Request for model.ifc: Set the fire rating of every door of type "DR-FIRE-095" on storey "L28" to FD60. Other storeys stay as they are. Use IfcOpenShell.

First a look at what the model holds.

```python
import ifcopenshell
import ifcopenshell.util.element

model = ifcopenshell.open("model.ifc")
print(model.schema)
storey = next(s for s in model.by_type("IfcBuildingStorey") if s.Name == "L28")
doors = [e for e in ifcopenshell.util.element.get_decomposition(storey) if e.is_a("IfcDoor")]
seen = {}
for e in doors:
    element_type = ifcopenshell.util.element.get_type(e)
    key = (element_type.Name if element_type != e and element_type else None, ifcopenshell.util.element.get_pset(e, "Pset_DoorCommon", "FireRating"))
    seen[key] = seen.get(key, 0) + 1
for (name, value), count in sorted(seen.items(), key=str):
    print(count, "x", name, "|", value)
```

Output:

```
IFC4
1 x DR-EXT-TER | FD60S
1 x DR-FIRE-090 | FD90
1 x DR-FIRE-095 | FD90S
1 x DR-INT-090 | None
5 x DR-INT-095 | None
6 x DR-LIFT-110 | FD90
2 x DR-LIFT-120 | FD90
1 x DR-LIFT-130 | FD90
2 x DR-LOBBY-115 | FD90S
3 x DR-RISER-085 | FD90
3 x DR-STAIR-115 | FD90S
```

```python
import ifcopenshell
import ifcopenshell.api.pset
import ifcopenshell.util.element

model = ifcopenshell.open("model.ifc")

storey = next(s for s in model.by_type("IfcBuildingStorey") if s.Name == "L28")
doors = [e for e in ifcopenshell.util.element.get_decomposition(storey) if e.is_a("IfcDoor")]

count = 0
for e in doors:
    element_type = ifcopenshell.util.element.get_type(e)
    if element_type in (None, e) or element_type.Name != "DR-FIRE-095":
        continue
    found = ifcopenshell.util.element.get_pset(e, "Pset_DoorCommon", should_inherit=False)
    if found:
        pset = model.by_id(found["id"])
        if len(ifcopenshell.util.element.get_elements_by_pset(pset)) > 1:
            pset = ifcopenshell.api.pset.unshare_pset(model, products=[e], pset=pset)[0]
    else:
        pset = ifcopenshell.api.pset.add_pset(model, product=e, name="Pset_DoorCommon")
    ifcopenshell.api.pset.edit_pset(model, pset=pset, properties={"FireRating": "FD60"})
    count += 1

print(count, "doors updated")

model.write("model_v2.ifc")
```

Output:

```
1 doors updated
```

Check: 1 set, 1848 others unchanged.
